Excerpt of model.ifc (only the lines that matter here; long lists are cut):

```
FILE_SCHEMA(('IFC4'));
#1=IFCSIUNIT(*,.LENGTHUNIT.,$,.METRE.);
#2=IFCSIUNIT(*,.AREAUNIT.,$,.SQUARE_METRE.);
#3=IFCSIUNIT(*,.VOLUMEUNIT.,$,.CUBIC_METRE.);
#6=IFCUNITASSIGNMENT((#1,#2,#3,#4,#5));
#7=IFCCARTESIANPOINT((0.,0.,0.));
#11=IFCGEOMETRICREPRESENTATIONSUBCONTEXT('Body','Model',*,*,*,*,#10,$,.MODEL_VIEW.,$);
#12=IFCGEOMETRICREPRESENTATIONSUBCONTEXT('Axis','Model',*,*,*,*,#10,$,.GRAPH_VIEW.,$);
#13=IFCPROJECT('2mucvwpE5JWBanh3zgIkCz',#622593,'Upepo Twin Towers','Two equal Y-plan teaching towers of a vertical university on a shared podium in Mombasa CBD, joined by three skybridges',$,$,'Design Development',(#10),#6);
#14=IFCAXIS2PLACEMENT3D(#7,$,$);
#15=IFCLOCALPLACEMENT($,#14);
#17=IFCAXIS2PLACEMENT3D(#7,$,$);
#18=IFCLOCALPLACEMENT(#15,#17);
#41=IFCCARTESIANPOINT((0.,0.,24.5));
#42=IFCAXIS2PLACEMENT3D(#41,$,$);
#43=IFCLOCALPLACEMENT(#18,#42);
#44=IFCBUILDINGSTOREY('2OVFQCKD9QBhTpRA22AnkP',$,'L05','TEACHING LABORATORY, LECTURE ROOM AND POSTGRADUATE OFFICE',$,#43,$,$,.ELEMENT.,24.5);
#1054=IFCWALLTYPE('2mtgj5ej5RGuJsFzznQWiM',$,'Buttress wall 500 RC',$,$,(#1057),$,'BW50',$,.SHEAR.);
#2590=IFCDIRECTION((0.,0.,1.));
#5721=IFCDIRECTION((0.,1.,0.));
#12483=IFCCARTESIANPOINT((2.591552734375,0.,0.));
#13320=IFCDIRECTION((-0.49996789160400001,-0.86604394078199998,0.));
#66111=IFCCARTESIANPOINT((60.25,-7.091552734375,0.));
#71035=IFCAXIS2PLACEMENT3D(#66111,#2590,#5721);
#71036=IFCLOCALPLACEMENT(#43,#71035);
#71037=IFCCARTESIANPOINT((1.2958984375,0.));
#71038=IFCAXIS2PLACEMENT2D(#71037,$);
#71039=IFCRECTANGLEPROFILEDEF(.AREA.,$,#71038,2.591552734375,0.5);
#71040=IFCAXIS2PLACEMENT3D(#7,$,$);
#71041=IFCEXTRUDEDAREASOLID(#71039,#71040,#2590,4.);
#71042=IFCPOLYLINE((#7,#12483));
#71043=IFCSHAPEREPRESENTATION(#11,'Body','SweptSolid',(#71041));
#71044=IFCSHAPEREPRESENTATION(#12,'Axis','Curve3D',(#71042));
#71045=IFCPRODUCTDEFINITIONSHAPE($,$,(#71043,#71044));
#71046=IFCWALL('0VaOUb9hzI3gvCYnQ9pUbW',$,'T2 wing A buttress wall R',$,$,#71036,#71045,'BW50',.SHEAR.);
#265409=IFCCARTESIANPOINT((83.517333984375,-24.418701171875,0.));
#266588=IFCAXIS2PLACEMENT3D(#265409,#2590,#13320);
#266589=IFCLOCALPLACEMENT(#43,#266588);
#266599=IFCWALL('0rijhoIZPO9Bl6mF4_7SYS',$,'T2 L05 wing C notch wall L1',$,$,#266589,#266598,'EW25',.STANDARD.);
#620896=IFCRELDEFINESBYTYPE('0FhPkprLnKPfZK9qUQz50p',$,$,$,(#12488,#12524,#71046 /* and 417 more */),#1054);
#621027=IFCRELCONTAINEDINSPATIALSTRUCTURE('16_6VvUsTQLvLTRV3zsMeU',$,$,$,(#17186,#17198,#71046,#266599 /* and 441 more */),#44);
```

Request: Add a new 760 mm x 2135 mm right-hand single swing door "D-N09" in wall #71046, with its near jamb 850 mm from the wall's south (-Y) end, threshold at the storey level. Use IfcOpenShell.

```python
import numpy as np
import ifcopenshell
import ifcopenshell.api.feature
import ifcopenshell.api.geometry
import ifcopenshell.api.root
import ifcopenshell.api.spatial
import ifcopenshell.geom
import ifcopenshell.util.element
import ifcopenshell.util.placement
import ifcopenshell.util.representation
import ifcopenshell.util.shape
import ifcopenshell.util.unit

model = ifcopenshell.open("model.ifc")
unit_scale = ifcopenshell.util.unit.calculate_unit_scale(model)
settings = ifcopenshell.geom.settings()


def volume(element):
    """Net volume in cubic metres, openings subtracted."""
    shape = ifcopenshell.geom.create_shape(settings, element)
    return ifcopenshell.util.shape.get_volume(shape.geometry)


wall = model.by_id(71046)
storey = ifcopenshell.util.element.get_container(wall, ifc_class="IfcBuildingStorey")
context = ifcopenshell.util.representation.get_context(model, "Model", "Body", "MODEL_VIEW")
before = volume(wall)

width, height, from_end, sill = 0.76, 2.135, 0.85, 0.0  # metres

# The wall runs along its own X axis, and the end named is its -X end.
wall_shape = ifcopenshell.geom.create_shape(settings, wall)
x, y, z = ifcopenshell.util.shape.get_vertices(wall_shape.geometry).T
start = x.min() + from_end
face, thickness = float(y.min()), float(y.max() - y.min())
wall_matrix = ifcopenshell.util.placement.get_local_placement(wall.ObjectPlacement)
level = ifcopenshell.util.placement.get_local_placement(storey.ObjectPlacement)[2, 3]


def in_wall(x, y):
    """Placement at x, y metres in the wall's axes, at sill height."""
    matrix = wall_matrix.copy()
    matrix[:, 3] = wall_matrix @ np.array([x / unit_scale, y / unit_scale, 0.0, 1.0])
    matrix[2, 3] = level + sill / unit_scale
    return matrix


# Opening: a box that overshoots both wall faces by 50 mm.
opening = ifcopenshell.api.root.create_entity(model, ifc_class="IfcOpeningElement", predefined_type="OPENING")
box = ifcopenshell.api.geometry.add_wall_representation(
    model, context=context, length=width, height=height, thickness=thickness + 0.1
)
ifcopenshell.api.geometry.assign_representation(model, product=opening, representation=box)
ifcopenshell.api.geometry.edit_object_placement(model, product=opening, matrix=in_wall(start, face - 0.05), is_si=False)
ifcopenshell.api.feature.add_feature(model, feature=opening, element=wall)

door = ifcopenshell.api.root.create_entity(model, ifc_class="IfcDoor", name="D-N09", predefined_type="DOOR")
door.OverallWidth, door.OverallHeight = width / unit_scale, height / unit_scale
door.OperationType = "SINGLE_SWING_RIGHT"
body = ifcopenshell.api.geometry.add_door_representation(
    model,
    context=context,
    overall_width=door.OverallWidth,
    overall_height=door.OverallHeight,
    operation_type="SINGLE_SWING_RIGHT",
    lining_properties={"LiningDepth": thickness / unit_scale, "ThresholdDepth": thickness / unit_scale},
)
ifcopenshell.api.geometry.assign_representation(model, product=door, representation=body)
ifcopenshell.api.spatial.assign_container(model, products=[door], relating_structure=storey)
ifcopenshell.api.feature.add_filling(model, opening=opening, element=door)

# The lining spans the wall, so the door starts at the wall face.
ifcopenshell.api.geometry.edit_object_placement(model, product=door, matrix=in_wall(start, face), is_si=False)

after = volume(wall)

print(f"wall volume {before:.3f} -> {after:.3f} m3")

model.write("model-out.ifc")
```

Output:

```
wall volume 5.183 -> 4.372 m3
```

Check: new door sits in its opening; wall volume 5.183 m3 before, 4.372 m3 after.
